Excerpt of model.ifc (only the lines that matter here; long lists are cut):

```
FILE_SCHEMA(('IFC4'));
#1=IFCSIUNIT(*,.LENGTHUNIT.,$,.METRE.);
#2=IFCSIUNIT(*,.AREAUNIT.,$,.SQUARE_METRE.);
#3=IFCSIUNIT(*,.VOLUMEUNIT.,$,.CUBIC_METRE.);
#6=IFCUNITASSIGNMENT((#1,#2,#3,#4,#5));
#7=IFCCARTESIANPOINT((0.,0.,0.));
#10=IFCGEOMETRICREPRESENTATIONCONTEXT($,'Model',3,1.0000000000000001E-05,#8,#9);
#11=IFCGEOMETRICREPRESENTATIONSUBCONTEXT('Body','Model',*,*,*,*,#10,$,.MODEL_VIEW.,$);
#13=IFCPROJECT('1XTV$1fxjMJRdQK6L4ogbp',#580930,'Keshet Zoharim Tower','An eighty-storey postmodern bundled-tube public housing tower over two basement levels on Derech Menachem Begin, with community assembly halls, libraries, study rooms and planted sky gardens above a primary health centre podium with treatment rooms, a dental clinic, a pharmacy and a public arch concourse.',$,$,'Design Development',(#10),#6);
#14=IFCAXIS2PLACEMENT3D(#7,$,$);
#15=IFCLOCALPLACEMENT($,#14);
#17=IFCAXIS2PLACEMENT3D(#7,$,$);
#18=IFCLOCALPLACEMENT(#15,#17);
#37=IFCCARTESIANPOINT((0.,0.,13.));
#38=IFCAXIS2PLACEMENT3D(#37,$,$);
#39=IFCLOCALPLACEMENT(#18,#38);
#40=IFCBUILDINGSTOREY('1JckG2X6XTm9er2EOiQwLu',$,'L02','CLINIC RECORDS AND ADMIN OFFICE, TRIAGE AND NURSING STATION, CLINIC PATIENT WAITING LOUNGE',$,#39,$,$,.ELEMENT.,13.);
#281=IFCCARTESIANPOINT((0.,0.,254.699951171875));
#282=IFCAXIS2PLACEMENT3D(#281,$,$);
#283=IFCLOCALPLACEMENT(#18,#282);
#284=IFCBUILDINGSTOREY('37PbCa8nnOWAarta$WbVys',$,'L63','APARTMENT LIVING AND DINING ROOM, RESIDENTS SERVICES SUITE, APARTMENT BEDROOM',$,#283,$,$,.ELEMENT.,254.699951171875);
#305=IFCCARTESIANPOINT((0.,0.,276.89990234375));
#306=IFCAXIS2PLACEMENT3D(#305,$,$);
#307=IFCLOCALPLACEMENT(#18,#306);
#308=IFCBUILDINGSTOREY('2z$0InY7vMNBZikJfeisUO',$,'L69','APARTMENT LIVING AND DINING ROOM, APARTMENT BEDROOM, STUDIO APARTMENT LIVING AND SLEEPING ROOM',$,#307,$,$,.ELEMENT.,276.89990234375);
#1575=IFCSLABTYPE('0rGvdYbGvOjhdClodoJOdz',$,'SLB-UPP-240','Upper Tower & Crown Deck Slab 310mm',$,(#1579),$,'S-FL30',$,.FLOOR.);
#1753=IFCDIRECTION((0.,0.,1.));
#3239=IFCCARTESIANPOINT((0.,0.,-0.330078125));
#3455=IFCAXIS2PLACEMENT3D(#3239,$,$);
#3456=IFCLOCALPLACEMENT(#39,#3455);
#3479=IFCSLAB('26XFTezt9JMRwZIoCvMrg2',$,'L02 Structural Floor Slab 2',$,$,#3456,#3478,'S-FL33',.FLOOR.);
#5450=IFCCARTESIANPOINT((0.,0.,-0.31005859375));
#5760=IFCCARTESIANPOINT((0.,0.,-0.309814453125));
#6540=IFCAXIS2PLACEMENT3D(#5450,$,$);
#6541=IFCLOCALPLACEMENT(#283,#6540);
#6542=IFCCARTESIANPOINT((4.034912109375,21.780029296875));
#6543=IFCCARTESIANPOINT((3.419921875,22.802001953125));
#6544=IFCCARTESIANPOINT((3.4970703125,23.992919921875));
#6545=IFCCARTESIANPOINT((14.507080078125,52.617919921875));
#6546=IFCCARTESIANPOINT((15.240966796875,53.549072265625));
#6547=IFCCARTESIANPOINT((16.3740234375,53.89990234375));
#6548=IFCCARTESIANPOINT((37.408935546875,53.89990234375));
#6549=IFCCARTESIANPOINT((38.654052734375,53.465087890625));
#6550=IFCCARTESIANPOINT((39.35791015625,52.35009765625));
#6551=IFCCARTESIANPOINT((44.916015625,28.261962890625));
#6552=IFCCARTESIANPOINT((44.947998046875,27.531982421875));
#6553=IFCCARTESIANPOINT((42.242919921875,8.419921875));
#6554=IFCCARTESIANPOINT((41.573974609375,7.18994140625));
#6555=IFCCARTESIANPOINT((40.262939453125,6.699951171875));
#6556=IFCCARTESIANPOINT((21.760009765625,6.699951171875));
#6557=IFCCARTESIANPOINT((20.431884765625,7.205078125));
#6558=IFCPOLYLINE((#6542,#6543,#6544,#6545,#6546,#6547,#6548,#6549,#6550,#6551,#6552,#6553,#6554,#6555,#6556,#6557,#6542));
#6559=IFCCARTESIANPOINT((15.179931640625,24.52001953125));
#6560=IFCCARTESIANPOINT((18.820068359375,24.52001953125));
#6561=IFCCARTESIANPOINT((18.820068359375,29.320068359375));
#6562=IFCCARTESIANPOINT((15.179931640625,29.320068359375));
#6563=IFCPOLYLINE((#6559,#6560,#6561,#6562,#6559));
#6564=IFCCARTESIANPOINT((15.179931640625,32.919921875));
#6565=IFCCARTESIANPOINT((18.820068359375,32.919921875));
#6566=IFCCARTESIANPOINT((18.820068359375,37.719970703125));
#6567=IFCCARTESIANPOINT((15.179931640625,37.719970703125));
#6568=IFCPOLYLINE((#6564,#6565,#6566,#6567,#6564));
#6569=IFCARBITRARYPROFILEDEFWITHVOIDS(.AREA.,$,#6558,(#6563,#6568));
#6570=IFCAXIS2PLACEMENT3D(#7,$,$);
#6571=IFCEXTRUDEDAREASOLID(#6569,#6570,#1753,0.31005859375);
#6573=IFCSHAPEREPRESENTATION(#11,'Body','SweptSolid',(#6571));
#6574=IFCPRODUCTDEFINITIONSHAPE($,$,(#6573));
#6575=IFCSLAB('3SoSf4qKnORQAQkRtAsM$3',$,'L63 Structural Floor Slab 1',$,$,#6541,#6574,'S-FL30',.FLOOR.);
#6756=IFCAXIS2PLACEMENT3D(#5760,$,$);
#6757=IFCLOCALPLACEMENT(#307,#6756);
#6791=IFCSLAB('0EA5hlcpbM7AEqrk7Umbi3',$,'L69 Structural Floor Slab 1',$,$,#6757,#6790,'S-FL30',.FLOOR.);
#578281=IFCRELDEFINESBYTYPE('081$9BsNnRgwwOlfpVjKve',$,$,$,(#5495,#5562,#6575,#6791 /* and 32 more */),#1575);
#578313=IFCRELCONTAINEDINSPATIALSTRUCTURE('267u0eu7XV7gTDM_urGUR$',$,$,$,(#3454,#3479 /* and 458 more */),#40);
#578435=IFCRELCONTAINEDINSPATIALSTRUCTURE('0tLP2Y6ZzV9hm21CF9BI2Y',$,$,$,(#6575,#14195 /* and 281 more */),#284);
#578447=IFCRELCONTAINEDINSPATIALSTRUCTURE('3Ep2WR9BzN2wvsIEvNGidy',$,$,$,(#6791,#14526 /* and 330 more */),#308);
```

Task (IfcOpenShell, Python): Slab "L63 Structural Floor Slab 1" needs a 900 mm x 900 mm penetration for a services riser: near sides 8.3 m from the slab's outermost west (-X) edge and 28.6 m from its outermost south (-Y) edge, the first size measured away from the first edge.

```python
import numpy as np
import ifcopenshell
import ifcopenshell.api.feature
import ifcopenshell.api.geometry
import ifcopenshell.api.root
import ifcopenshell.geom
import ifcopenshell.util.placement
import ifcopenshell.util.representation
import ifcopenshell.util.shape
import ifcopenshell.util.unit

model = ifcopenshell.open("model.ifc")
unit_scale = ifcopenshell.util.unit.calculate_unit_scale(model)
settings = ifcopenshell.geom.settings()


def volume(element):
    """Net volume in cubic metres, openings subtracted."""
    shape = ifcopenshell.geom.create_shape(settings, element)
    return ifcopenshell.util.shape.get_volume(shape.geometry)


slab = model.by_guid("3SoSf4qKnORQAQkRtAsM$3")
before = volume(slab)

# Extent in the slab's own axes, in metres. The edges named are its -X and -Y sides.
slab_shape = ifcopenshell.geom.create_shape(settings, slab)
vertices = ifcopenshell.util.shape.get_vertices(slab_shape.geometry)
x_min, y_min, bottom = vertices.min(axis=0)
top = vertices[:, 2].max()

opening = ifcopenshell.api.root.create_entity(model, ifc_class="IfcOpeningElement", name="Services riser opening", predefined_type="OPENING")
context = ifcopenshell.util.representation.get_context(model, "Model", "Body", "MODEL_VIEW")
width, depth = 0.9, 0.9
outline = [(0.0, 0.0), (width, 0.0), (width, depth), (0.0, depth), (0.0, 0.0)]
# Overshoot both faces by 50 mm so the cut is clean.
shape = ifcopenshell.api.geometry.add_slab_representation(
    model, context=context, depth=top - bottom + 0.1, polyline=outline
)
ifcopenshell.api.geometry.assign_representation(model, product=opening, representation=shape)

matrix = ifcopenshell.util.placement.get_local_placement(slab.ObjectPlacement)
matrix[:, 3] = matrix @ np.append(np.array([x_min + 8.3, y_min + 28.6, bottom - 0.05]) / unit_scale, 1.0)
ifcopenshell.api.geometry.edit_object_placement(model, product=opening, matrix=matrix, is_si=False)
ifcopenshell.api.feature.add_feature(model, feature=opening, element=slab)

after = volume(slab)

print(f"slab volume {before:.3f} -> {after:.3f} m3")

model.write("model-out.ifc")
```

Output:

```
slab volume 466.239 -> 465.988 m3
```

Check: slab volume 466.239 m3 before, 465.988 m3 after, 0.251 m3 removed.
